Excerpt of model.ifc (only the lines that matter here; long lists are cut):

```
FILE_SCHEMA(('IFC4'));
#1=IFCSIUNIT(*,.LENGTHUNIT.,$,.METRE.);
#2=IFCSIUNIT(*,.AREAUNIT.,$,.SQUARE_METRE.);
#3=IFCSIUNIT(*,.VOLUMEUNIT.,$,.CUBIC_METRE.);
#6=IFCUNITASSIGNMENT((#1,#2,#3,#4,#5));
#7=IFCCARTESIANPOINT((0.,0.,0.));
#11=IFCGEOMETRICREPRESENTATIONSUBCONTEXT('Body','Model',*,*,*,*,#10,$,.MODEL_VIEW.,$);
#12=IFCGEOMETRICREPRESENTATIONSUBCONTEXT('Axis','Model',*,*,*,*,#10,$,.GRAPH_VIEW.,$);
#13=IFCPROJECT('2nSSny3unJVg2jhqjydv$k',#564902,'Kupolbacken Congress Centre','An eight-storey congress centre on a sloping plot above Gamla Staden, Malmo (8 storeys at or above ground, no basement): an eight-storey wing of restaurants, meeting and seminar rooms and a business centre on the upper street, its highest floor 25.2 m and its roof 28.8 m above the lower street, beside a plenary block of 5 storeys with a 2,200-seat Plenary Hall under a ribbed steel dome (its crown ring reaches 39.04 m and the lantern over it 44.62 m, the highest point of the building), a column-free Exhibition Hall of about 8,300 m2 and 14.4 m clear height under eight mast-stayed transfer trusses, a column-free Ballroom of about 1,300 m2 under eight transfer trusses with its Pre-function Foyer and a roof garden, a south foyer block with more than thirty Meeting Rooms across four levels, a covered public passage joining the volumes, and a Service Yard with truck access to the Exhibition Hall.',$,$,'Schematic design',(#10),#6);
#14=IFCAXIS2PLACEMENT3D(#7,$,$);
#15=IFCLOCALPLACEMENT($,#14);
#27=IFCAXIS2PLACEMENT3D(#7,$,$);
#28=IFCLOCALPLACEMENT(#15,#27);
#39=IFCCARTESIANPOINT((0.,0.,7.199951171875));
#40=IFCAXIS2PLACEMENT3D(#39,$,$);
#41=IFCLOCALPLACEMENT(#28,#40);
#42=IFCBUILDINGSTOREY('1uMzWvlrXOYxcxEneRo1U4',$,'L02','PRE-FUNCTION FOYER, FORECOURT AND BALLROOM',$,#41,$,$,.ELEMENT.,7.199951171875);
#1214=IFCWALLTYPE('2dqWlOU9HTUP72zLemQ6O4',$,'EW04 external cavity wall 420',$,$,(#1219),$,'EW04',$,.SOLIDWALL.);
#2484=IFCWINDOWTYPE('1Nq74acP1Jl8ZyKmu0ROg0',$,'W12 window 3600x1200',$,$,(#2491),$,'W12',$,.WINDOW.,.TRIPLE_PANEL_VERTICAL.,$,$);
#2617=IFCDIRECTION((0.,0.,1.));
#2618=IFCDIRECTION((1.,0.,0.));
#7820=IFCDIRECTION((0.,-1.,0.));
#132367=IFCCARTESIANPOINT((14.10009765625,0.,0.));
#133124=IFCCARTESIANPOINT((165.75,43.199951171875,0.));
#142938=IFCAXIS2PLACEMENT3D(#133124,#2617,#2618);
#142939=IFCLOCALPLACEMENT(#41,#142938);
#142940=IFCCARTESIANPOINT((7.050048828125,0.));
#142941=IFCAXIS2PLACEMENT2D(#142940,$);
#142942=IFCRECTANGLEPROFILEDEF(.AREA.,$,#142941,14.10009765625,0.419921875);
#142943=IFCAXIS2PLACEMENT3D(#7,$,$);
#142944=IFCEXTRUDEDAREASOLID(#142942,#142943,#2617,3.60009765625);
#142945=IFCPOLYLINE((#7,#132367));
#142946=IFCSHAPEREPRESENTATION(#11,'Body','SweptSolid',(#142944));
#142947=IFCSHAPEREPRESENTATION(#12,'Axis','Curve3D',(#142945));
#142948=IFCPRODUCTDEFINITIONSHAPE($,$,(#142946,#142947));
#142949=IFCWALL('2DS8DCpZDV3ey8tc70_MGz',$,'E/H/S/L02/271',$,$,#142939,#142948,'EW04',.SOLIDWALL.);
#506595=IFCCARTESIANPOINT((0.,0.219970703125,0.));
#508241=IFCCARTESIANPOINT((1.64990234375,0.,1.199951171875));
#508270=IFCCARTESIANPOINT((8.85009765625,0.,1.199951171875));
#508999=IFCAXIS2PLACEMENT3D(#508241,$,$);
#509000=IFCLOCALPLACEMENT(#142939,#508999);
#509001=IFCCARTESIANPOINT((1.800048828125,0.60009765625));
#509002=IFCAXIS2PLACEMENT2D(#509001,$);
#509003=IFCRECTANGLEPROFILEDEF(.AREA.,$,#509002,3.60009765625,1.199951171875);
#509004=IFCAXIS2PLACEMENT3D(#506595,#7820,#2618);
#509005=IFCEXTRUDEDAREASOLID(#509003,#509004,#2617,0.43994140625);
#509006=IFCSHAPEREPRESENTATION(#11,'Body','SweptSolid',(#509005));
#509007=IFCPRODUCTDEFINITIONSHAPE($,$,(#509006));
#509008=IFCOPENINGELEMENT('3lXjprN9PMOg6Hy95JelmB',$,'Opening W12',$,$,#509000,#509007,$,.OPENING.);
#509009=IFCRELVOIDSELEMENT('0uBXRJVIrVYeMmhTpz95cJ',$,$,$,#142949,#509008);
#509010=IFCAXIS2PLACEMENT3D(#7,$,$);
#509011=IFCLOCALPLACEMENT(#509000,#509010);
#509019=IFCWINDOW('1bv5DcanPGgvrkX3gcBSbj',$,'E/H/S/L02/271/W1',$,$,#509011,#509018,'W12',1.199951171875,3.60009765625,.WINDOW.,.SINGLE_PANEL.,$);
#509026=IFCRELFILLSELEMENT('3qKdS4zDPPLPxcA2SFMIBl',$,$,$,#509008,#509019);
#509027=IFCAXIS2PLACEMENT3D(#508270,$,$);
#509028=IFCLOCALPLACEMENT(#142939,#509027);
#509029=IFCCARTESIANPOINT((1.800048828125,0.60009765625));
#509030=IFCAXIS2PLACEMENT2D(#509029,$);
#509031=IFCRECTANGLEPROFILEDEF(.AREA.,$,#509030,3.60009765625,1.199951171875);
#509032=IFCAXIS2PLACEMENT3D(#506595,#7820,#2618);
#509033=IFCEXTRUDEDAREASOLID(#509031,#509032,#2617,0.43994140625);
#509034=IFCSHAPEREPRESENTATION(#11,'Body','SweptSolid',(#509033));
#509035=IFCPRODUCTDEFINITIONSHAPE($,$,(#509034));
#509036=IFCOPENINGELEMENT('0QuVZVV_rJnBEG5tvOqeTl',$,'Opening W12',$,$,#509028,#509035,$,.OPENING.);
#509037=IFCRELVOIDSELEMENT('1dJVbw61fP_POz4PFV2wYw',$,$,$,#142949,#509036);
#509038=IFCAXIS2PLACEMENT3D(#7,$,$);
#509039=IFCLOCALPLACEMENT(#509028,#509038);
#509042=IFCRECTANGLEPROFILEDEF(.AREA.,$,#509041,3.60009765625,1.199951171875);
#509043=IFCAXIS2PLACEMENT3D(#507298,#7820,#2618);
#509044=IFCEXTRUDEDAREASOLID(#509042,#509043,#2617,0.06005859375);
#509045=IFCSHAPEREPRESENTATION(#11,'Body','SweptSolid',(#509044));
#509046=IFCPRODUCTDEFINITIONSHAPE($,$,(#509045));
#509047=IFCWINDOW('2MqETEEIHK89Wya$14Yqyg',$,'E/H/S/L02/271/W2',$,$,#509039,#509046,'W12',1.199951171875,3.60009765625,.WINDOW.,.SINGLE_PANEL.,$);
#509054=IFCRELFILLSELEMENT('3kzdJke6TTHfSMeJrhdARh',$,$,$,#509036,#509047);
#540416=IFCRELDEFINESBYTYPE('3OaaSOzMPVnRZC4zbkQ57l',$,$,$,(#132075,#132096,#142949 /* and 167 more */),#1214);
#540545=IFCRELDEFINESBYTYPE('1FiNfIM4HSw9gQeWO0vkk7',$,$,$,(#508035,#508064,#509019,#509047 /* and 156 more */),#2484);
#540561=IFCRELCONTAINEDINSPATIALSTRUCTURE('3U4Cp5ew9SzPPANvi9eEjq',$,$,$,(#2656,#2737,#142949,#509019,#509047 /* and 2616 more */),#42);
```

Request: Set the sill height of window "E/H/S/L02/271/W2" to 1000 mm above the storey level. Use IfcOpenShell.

```python
import numpy as np
import ifcopenshell
import ifcopenshell.api.geometry
import ifcopenshell.geom
import ifcopenshell.util.element
import ifcopenshell.util.placement
import ifcopenshell.util.shape
import ifcopenshell.util.unit

model = ifcopenshell.open("model.ifc")
unit_scale = ifcopenshell.util.unit.calculate_unit_scale(model)

window = model.by_guid("2MqETEEIHK89Wya$14Yqyg")
opening = window.FillsVoids[0].RelatingOpeningElement
storey = ifcopenshell.util.element.get_container(window, ifc_class="IfcBuildingStorey")
level = ifcopenshell.util.placement.get_local_placement(storey.ObjectPlacement)[2, 3]

# The opening's origin need not be at the sill, so measure its lowest point.
shape = ifcopenshell.geom.create_shape(ifcopenshell.geom.settings(), opening)
bottom = ifcopenshell.util.shape.get_shape_bottom_elevation(shape, shape.geometry) / unit_scale
dz = level + 1.0 - bottom

shift = np.array([0.0, 0.0, dz])
# The window is placed relative to its opening, so it follows when the opening moves.
matrix = ifcopenshell.util.placement.get_local_placement(opening.ObjectPlacement)
matrix[:3, 3] += shift
ifcopenshell.api.geometry.edit_object_placement(
    model, product=opening, matrix=matrix, is_si=False, should_transform_children=True
)

print(f"moved by {dz * unit_scale:+.3f} m")

model.write("model_v2.ifc")
```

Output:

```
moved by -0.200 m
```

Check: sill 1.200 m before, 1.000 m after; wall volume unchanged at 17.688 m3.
